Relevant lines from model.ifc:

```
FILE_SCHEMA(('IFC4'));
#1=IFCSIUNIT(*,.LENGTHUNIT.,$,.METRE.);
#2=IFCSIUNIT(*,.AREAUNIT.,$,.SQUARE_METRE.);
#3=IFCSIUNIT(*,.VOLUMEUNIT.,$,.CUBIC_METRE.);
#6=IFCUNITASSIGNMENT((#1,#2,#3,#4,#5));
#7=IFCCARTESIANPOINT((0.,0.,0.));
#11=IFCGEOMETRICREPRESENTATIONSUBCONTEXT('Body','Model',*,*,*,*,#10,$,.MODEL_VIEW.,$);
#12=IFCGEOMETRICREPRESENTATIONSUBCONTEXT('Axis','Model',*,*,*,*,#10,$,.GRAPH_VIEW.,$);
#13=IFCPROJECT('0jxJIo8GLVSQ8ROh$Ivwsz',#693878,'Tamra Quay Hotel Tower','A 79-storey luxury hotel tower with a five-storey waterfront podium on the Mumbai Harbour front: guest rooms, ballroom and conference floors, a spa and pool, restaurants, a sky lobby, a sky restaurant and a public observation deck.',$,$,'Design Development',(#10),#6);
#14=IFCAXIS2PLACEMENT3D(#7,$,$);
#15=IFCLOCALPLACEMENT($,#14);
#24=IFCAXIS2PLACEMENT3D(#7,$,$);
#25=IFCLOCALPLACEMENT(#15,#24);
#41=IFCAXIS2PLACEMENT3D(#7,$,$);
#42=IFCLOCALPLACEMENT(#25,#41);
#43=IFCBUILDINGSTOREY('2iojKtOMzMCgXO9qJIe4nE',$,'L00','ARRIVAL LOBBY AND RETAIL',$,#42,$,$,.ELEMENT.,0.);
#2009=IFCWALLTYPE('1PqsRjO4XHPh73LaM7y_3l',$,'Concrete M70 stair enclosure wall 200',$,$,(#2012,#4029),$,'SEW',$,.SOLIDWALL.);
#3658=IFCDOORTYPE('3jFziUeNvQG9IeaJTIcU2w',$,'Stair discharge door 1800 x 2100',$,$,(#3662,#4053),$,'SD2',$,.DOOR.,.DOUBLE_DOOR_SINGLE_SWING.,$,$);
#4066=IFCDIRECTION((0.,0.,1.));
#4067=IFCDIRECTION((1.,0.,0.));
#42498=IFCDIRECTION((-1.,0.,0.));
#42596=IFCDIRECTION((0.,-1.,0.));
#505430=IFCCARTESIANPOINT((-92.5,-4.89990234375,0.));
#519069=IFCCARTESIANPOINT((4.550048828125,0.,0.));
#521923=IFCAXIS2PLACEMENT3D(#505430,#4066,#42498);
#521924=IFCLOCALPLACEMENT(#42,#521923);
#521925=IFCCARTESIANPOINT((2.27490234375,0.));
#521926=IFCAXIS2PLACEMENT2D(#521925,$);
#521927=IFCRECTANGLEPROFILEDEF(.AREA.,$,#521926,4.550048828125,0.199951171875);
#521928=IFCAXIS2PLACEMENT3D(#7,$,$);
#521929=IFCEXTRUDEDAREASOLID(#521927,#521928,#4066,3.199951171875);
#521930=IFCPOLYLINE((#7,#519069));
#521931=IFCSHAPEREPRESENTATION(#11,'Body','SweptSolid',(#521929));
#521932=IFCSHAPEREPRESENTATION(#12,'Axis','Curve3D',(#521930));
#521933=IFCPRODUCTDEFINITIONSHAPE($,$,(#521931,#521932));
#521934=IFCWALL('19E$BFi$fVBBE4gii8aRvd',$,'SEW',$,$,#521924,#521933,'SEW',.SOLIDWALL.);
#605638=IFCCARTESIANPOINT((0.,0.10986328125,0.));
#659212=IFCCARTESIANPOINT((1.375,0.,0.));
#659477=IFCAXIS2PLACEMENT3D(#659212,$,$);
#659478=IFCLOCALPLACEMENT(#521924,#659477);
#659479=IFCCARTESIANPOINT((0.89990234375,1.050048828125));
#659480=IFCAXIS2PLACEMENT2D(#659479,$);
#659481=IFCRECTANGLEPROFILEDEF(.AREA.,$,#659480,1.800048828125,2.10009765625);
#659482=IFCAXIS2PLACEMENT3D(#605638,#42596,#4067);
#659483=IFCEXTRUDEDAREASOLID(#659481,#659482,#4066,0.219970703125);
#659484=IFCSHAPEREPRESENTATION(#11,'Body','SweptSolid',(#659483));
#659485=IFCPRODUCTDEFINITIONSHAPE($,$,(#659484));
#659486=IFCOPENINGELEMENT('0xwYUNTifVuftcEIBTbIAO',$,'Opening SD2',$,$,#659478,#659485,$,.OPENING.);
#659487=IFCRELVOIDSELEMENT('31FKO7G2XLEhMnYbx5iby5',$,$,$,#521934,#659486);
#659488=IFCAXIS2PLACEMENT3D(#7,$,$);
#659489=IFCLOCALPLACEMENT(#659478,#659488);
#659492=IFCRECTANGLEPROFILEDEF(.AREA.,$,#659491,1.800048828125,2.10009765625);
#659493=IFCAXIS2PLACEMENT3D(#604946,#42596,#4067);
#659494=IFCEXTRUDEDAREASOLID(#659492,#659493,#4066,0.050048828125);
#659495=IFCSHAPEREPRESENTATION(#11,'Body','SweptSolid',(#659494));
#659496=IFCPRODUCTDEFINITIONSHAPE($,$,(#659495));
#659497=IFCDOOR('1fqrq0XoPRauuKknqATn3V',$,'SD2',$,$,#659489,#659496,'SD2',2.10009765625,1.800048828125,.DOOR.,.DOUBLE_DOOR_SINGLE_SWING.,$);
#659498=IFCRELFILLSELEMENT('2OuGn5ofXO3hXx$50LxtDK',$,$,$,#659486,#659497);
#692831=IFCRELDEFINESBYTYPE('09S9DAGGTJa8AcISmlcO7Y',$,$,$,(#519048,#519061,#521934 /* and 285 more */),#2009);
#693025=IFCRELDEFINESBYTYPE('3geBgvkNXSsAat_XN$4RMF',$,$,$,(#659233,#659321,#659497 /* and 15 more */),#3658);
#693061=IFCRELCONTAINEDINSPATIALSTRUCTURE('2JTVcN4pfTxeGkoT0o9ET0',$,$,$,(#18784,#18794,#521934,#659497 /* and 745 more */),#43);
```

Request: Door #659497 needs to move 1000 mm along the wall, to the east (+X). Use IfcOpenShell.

```python
import ifcopenshell
import ifcopenshell.api.geometry
import ifcopenshell.util.placement

model = ifcopenshell.open("model.ifc")

door = model.by_id(659497)
opening = door.FillsVoids[0].RelatingOpeningElement
wall = opening.VoidsElements[0].RelatingBuildingElement

wall_matrix = ifcopenshell.util.placement.get_local_placement(wall.ObjectPlacement)
shift = wall_matrix[:3, 0] * -1.0
before = ifcopenshell.util.placement.get_local_placement(door.ObjectPlacement)[:3, 3].copy()

# The door is placed relative to its opening, so it follows when the opening moves.
matrix = ifcopenshell.util.placement.get_local_placement(opening.ObjectPlacement)
matrix[:3, 3] += shift
ifcopenshell.api.geometry.edit_object_placement(
    model, product=opening, matrix=matrix, is_si=False, should_transform_children=True
)

after = ifcopenshell.util.placement.get_local_placement(door.ObjectPlacement)[:3, 3]
print("door moved by", (after - before).round(3) + 0.0)

model.write("model_rev.ifc")
```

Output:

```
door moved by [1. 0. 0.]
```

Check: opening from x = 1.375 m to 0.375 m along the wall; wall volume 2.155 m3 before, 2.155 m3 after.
